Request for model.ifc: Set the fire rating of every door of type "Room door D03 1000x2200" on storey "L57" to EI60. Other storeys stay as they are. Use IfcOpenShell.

First a look at what the model holds.

```python
import ifcopenshell
import ifcopenshell.util.element

model = ifcopenshell.open("model.ifc")
print(model.schema)
storey = next(s for s in model.by_type("IfcBuildingStorey") if s.Name == "L57")
doors = [e for e in ifcopenshell.util.element.get_decomposition(storey) if e.is_a("IfcDoor")]
seen = {}
for e in doors:
    element_type = ifcopenshell.util.element.get_type(e)
    key = (element_type.Name if element_type != e and element_type else None, ifcopenshell.util.element.get_pset(e, "Pset_DoorCommon", "FireRating"))
    seen[key] = seen.get(key, 0) + 1
for (name, value), count in sorted(seen.items(), key=str):
    print(count, "x", name, "|", value)
```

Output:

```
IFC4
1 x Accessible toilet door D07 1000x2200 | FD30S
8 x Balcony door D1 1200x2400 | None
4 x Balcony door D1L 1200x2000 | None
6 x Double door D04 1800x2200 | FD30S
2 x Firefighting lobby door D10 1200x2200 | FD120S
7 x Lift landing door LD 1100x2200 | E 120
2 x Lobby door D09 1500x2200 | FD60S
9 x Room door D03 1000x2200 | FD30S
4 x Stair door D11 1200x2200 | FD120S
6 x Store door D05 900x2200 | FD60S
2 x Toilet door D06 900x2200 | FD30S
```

```python
import ifcopenshell
import ifcopenshell.api.pset
import ifcopenshell.util.element

model = ifcopenshell.open("model.ifc")

storey = next(s for s in model.by_type("IfcBuildingStorey") if s.Name == "L57")
doors = [e for e in ifcopenshell.util.element.get_decomposition(storey) if e.is_a("IfcDoor")]

count = 0
for e in doors:
    element_type = ifcopenshell.util.element.get_type(e)
    if element_type in (None, e) or element_type.Name != "Room door D03 1000x2200":
        continue
    # add_pset returns the element's existing set when there is one.
    pset = ifcopenshell.api.pset.add_pset(model, product=e, name="Pset_DoorCommon")
    ifcopenshell.api.pset.edit_pset(model, pset=pset, properties={"FireRating": "EI60"})
    count += 1

print(count, "doors updated")

model.write("model_rev.ifc")
```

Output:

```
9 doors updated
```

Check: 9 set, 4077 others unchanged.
